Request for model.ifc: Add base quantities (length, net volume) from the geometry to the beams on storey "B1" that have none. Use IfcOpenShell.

First a look at what the model holds.

```python
import ifcopenshell
import ifcopenshell.util.element
import ifcopenshell.util.unit

model = ifcopenshell.open("model.ifc")
print(model.schema)
for unit_type in ("LENGTHUNIT", "AREAUNIT", "VOLUMEUNIT"):
    print(unit_type, ifcopenshell.util.unit.calculate_unit_scale(model, unit_type))
storey = next(s for s in model.by_type("IfcBuildingStorey") if s.Name == "B1")
beams = [e for e in ifcopenshell.util.element.get_decomposition(storey) if e.is_a("IfcBeam")]
for e in sorted(beams, key=lambda e: e.id()):
    print(e.id(), e.is_a(), e.Name, list(ifcopenshell.util.element.get_psets(e, qtos_only=True)), sep=" | ")
```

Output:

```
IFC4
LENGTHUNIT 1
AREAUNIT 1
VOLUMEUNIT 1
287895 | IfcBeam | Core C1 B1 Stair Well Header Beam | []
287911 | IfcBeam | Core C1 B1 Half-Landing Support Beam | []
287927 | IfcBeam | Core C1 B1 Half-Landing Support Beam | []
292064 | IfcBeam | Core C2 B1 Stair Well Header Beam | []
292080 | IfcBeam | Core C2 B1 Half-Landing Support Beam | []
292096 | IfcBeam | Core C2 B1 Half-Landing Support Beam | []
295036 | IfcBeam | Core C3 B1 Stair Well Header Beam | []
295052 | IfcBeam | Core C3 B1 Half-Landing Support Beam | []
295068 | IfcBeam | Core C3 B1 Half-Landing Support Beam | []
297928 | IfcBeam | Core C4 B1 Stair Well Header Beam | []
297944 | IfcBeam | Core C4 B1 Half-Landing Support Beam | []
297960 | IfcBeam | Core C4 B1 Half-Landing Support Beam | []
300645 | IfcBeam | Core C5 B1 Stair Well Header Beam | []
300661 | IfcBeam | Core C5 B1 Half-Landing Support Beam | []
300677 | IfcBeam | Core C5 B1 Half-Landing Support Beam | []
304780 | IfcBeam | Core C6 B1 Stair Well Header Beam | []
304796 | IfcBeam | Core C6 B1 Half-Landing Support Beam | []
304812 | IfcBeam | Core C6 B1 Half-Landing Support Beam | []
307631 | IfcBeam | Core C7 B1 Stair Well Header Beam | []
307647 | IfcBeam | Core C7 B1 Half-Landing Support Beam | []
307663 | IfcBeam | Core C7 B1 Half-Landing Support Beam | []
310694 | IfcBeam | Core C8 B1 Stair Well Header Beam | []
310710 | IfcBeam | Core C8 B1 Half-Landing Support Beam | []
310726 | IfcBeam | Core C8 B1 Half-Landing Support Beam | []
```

```python
import ifcopenshell
import ifcopenshell.api.pset
import ifcopenshell.geom
import ifcopenshell.util.element
import ifcopenshell.util.shape
import ifcopenshell.util.unit

model = ifcopenshell.open("model.ifc")
unit_scale = ifcopenshell.util.unit.calculate_unit_scale(model)
volume_scale = ifcopenshell.util.unit.calculate_unit_scale(model, "VOLUMEUNIT")
settings = ifcopenshell.geom.settings()

storey = next(s for s in model.by_type("IfcBuildingStorey") if s.Name == "B1")
beams = [e for e in ifcopenshell.util.element.get_decomposition(storey) if e.is_a("IfcBeam")]

for e in sorted(beams, key=lambda e: e.id()):
    if ifcopenshell.util.element.get_psets(e, qtos_only=True, should_inherit=False):
        continue
    # Geometry comes back in metres, in the element's own axes.
    shape = ifcopenshell.geom.create_shape(settings, e)
    values = {
        "Length": ifcopenshell.util.shape.get_max_xyz(shape.geometry) / unit_scale,
        "NetVolume": ifcopenshell.util.shape.get_volume(shape.geometry) / volume_scale,
    }
    qto = ifcopenshell.api.pset.add_qto(model, product=e, name="Qto_BeamBaseQuantities")
    ifcopenshell.api.pset.edit_qto(model, qto=qto, properties=values)
    print(e.id(), {k: round(v, 3) for k, v in values.items()})

model.write("model_rev.ifc")
```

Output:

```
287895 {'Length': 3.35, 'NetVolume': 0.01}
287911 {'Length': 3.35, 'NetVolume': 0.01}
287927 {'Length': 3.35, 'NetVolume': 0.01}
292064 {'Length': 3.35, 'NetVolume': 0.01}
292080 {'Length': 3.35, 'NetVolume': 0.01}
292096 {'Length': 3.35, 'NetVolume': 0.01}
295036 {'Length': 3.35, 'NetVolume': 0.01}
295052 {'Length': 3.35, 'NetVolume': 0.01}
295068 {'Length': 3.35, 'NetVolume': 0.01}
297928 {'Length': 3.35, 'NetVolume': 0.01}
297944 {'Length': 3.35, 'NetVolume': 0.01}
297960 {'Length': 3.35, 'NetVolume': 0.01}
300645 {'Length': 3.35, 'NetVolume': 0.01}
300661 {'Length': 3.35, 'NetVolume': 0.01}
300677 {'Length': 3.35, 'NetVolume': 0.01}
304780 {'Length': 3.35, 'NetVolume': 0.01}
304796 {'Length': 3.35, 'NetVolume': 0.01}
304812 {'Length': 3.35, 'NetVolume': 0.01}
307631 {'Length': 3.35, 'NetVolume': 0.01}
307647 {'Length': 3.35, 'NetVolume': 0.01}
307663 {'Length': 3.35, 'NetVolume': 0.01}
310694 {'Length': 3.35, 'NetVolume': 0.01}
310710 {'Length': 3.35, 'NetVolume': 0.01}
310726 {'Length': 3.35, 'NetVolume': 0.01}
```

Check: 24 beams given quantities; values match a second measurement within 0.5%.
